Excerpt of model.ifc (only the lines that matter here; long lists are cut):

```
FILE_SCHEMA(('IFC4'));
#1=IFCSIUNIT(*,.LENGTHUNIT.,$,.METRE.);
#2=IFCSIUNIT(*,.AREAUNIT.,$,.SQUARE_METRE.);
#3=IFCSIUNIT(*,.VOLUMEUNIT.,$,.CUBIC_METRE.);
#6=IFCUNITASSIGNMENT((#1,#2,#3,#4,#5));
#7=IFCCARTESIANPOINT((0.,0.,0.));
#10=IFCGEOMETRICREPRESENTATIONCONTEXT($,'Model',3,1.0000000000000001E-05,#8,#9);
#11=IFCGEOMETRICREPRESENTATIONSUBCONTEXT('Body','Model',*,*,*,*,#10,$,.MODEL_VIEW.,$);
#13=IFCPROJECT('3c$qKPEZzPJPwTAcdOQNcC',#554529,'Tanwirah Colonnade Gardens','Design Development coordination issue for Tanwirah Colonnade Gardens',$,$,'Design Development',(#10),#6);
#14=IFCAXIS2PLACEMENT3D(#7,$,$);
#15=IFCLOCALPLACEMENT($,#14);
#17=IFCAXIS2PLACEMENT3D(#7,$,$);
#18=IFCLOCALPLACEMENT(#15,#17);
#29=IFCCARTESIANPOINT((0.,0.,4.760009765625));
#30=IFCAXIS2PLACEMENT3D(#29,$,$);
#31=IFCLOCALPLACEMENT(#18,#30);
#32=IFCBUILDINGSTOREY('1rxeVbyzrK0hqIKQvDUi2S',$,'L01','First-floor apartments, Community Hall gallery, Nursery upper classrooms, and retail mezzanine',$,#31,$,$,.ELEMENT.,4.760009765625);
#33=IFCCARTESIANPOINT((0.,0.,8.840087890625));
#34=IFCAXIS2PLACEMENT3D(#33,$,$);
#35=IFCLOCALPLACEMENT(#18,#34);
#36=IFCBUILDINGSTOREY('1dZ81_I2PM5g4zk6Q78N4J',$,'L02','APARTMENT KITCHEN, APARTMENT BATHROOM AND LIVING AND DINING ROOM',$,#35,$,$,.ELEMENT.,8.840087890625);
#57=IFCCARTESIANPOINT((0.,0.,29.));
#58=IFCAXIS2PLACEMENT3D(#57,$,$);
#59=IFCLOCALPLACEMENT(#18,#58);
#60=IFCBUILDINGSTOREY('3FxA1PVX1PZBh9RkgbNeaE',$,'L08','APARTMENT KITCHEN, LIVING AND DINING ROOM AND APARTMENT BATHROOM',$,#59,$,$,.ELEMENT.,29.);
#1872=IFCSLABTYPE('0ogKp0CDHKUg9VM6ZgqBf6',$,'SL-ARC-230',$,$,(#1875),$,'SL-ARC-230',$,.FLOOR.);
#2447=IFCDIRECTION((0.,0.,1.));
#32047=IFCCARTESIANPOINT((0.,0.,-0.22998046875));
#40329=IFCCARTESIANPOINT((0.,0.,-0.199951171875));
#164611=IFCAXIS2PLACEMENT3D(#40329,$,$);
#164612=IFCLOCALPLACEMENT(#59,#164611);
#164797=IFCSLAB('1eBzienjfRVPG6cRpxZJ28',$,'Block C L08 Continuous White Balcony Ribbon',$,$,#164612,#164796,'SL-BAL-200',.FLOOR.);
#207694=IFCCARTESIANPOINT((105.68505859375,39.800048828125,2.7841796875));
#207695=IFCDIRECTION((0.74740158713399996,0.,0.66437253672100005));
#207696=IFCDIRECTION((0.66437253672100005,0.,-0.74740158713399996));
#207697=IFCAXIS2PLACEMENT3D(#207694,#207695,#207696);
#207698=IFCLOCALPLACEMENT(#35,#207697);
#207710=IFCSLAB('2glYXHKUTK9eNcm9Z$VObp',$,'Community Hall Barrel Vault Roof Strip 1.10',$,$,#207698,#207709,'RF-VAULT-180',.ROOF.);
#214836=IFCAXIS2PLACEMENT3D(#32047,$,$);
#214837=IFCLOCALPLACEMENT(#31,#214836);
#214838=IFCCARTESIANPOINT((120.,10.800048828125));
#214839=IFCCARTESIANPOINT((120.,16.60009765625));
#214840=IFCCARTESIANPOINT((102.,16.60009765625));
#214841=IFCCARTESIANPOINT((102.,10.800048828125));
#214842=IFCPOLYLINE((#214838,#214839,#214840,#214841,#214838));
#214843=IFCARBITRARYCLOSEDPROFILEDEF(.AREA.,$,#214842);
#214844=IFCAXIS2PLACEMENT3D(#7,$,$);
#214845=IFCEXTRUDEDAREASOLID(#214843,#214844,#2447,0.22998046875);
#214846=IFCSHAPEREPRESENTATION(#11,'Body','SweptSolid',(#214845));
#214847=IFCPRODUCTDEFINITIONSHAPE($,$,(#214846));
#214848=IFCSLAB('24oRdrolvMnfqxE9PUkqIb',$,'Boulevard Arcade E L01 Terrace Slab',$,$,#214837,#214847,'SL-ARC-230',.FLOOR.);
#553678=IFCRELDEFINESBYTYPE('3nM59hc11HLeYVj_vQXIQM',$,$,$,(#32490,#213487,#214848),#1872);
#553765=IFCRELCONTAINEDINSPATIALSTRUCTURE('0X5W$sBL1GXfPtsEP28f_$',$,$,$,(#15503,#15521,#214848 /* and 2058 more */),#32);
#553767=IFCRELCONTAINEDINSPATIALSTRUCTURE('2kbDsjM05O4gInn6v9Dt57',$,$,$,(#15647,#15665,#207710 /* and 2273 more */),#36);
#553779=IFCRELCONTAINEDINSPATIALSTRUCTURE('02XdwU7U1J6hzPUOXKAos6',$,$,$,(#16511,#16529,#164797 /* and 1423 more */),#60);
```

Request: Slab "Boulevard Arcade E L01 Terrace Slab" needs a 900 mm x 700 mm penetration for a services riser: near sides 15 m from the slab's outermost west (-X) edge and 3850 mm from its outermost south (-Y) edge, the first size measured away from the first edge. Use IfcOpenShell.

```python
import numpy as np
import ifcopenshell
import ifcopenshell.api.feature
import ifcopenshell.api.geometry
import ifcopenshell.api.root
import ifcopenshell.geom
import ifcopenshell.util.placement
import ifcopenshell.util.representation
import ifcopenshell.util.shape
import ifcopenshell.util.unit

model = ifcopenshell.open("model.ifc")
unit_scale = ifcopenshell.util.unit.calculate_unit_scale(model)
settings = ifcopenshell.geom.settings()


def volume(element):
    """Net volume in cubic metres, openings subtracted."""
    shape = ifcopenshell.geom.create_shape(settings, element)
    return ifcopenshell.util.shape.get_volume(shape.geometry)


slab = model.by_id(214848)
before = volume(slab)

# Extent in the slab's own axes, in metres. The edges named are its -X and -Y sides.
slab_shape = ifcopenshell.geom.create_shape(settings, slab)
vertices = ifcopenshell.util.shape.get_vertices(slab_shape.geometry)
x_min, y_min, bottom = vertices.min(axis=0)
top = vertices[:, 2].max()

opening = ifcopenshell.api.root.create_entity(model, ifc_class="IfcOpeningElement", name="Services riser opening", predefined_type="OPENING")
context = ifcopenshell.util.representation.get_context(model, "Model", "Body", "MODEL_VIEW")
width, depth = 0.9, 0.7
outline = [(0.0, 0.0), (width, 0.0), (width, depth), (0.0, depth), (0.0, 0.0)]
# Overshoot both faces by 50 mm so the cut is clean.
shape = ifcopenshell.api.geometry.add_slab_representation(
    model, context=context, depth=top - bottom + 0.1, polyline=outline
)
ifcopenshell.api.geometry.assign_representation(model, product=opening, representation=shape)

matrix = ifcopenshell.util.placement.get_local_placement(slab.ObjectPlacement)
matrix[:, 3] = matrix @ np.append(np.array([x_min + 15, y_min + 3.85, bottom - 0.05]) / unit_scale, 1.0)
ifcopenshell.api.geometry.edit_object_placement(model, product=opening, matrix=matrix, is_si=False)
ifcopenshell.api.feature.add_feature(model, feature=opening, element=slab)

after = volume(slab)

print(f"slab volume {before:.3f} -> {after:.3f} m3")

model.write("model_edited.ifc")
```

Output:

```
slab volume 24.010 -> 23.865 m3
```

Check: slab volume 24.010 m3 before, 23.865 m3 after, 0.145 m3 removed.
